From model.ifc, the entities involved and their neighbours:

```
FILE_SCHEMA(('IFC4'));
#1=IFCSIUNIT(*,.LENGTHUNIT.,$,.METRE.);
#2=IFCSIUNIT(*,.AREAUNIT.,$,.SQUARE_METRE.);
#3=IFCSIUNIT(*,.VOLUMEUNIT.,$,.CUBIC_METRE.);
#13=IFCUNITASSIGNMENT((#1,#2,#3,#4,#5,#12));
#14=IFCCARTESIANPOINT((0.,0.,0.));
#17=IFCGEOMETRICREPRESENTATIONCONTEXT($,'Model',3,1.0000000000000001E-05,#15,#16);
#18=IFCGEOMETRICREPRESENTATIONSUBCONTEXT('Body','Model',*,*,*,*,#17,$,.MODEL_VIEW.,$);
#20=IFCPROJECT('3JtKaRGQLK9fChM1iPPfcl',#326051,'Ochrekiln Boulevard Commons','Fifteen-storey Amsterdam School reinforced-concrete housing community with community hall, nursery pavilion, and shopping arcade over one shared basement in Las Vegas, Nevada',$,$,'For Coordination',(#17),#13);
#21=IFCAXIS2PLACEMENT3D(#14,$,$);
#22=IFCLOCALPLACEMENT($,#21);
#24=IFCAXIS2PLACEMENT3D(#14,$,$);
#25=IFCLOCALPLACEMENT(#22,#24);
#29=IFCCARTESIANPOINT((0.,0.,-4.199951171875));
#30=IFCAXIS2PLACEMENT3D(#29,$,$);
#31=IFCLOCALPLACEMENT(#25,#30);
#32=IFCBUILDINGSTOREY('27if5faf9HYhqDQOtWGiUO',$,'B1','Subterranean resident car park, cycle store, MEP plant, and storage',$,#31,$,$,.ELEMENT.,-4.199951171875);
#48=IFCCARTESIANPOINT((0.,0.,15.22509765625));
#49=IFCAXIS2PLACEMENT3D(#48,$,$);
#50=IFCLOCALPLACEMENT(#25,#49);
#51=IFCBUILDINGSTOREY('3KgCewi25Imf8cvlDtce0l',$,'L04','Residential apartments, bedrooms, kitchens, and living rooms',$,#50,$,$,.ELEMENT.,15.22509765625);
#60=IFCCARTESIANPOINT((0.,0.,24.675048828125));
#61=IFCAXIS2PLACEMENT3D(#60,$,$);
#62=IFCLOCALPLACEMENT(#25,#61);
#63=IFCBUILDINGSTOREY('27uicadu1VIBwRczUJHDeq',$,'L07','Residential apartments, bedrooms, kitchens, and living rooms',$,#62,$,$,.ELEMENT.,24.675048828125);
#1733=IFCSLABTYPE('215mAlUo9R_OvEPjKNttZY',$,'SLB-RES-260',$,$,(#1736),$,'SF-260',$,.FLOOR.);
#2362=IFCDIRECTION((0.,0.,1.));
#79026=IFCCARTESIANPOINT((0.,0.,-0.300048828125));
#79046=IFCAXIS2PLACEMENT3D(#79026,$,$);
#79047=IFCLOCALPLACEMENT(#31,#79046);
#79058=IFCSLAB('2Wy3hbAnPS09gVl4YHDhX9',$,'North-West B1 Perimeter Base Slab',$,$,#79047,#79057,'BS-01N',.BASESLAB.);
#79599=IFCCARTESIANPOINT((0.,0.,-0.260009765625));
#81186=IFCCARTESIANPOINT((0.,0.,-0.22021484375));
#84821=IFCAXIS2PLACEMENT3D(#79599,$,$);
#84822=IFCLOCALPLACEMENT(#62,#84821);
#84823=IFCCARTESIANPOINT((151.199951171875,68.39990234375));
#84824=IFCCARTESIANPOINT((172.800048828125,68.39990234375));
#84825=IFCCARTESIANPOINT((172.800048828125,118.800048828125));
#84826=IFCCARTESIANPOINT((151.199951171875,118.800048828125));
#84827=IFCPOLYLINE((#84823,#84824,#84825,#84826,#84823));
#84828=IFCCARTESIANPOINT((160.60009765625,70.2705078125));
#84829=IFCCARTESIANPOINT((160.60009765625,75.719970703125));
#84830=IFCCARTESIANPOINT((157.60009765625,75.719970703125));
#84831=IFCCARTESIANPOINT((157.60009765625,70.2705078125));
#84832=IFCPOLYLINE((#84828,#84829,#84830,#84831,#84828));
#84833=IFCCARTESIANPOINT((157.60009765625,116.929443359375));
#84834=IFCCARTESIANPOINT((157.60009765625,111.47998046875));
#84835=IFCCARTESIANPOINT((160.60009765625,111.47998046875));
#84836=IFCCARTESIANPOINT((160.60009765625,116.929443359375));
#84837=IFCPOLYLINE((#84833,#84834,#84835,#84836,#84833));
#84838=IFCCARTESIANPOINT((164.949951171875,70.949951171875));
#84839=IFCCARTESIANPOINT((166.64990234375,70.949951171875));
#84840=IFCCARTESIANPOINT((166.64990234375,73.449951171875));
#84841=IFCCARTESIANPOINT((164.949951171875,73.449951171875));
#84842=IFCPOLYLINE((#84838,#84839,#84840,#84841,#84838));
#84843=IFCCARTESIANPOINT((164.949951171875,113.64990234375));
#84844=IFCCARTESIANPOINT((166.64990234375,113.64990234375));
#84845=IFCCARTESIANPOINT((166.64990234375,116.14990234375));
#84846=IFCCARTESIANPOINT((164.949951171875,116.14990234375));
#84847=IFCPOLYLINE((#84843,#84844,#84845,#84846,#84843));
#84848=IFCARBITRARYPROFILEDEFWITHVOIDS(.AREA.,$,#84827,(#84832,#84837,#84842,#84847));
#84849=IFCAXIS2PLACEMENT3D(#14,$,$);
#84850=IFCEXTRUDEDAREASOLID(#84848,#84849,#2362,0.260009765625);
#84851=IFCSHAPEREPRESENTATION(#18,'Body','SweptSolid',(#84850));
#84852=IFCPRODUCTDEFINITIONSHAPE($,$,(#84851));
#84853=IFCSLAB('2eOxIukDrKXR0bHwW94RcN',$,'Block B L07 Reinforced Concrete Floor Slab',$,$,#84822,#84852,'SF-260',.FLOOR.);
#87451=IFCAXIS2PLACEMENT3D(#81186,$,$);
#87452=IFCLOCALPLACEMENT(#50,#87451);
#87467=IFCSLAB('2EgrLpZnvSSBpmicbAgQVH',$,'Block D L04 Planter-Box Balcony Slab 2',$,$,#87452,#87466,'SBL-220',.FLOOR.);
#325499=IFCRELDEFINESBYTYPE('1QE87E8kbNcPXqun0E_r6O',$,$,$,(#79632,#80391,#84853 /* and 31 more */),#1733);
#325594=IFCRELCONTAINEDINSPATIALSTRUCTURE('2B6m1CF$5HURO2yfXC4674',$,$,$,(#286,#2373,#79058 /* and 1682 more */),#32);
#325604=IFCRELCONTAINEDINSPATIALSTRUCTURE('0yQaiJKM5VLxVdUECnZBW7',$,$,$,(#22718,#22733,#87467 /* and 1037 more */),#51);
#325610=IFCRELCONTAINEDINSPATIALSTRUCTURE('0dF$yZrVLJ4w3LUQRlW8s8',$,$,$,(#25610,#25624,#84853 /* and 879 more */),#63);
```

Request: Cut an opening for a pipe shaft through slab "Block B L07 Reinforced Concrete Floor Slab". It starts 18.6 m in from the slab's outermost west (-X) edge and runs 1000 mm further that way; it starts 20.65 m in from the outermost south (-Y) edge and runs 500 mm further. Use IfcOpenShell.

```python
import numpy as np
import ifcopenshell
import ifcopenshell.api.feature
import ifcopenshell.api.geometry
import ifcopenshell.api.root
import ifcopenshell.geom
import ifcopenshell.util.placement
import ifcopenshell.util.representation
import ifcopenshell.util.shape
import ifcopenshell.util.unit

model = ifcopenshell.open("model.ifc")
unit_scale = ifcopenshell.util.unit.calculate_unit_scale(model)
settings = ifcopenshell.geom.settings()


def volume(element):
    """Net volume in cubic metres, openings subtracted."""
    shape = ifcopenshell.geom.create_shape(settings, element)
    return ifcopenshell.util.shape.get_volume(shape.geometry)


slab = model.by_guid("2eOxIukDrKXR0bHwW94RcN")
before = volume(slab)

# Extent in the slab's own axes, in metres. The edges named are its -X and -Y sides.
slab_shape = ifcopenshell.geom.create_shape(settings, slab)
vertices = ifcopenshell.util.shape.get_vertices(slab_shape.geometry)
x_min, y_min, bottom = vertices.min(axis=0)
top = vertices[:, 2].max()

opening = ifcopenshell.api.root.create_entity(model, ifc_class="IfcOpeningElement", name="Pipe shaft opening", predefined_type="OPENING")
context = ifcopenshell.util.representation.get_context(model, "Model", "Body", "MODEL_VIEW")
width, depth = 1, 0.5
outline = [(0.0, 0.0), (width, 0.0), (width, depth), (0.0, depth), (0.0, 0.0)]
# Overshoot both faces by 50 mm so the cut is clean.
shape = ifcopenshell.api.geometry.add_slab_representation(
    model, context=context, depth=top - bottom + 0.1, polyline=outline
)
ifcopenshell.api.geometry.assign_representation(model, product=opening, representation=shape)

matrix = ifcopenshell.util.placement.get_local_placement(slab.ObjectPlacement)
matrix[:, 3] = matrix @ np.append(np.array([x_min + 18.6, y_min + 20.65, bottom - 0.05]) / unit_scale, 1.0)
ifcopenshell.api.geometry.edit_object_placement(model, product=opening, matrix=matrix, is_si=False)
ifcopenshell.api.feature.add_feature(model, feature=opening, element=slab)

after = volume(slab)

print(f"slab volume {before:.3f} -> {after:.3f} m3")

model.write("model_edited.ifc")
```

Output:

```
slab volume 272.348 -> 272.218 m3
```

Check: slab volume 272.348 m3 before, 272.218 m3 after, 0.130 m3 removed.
